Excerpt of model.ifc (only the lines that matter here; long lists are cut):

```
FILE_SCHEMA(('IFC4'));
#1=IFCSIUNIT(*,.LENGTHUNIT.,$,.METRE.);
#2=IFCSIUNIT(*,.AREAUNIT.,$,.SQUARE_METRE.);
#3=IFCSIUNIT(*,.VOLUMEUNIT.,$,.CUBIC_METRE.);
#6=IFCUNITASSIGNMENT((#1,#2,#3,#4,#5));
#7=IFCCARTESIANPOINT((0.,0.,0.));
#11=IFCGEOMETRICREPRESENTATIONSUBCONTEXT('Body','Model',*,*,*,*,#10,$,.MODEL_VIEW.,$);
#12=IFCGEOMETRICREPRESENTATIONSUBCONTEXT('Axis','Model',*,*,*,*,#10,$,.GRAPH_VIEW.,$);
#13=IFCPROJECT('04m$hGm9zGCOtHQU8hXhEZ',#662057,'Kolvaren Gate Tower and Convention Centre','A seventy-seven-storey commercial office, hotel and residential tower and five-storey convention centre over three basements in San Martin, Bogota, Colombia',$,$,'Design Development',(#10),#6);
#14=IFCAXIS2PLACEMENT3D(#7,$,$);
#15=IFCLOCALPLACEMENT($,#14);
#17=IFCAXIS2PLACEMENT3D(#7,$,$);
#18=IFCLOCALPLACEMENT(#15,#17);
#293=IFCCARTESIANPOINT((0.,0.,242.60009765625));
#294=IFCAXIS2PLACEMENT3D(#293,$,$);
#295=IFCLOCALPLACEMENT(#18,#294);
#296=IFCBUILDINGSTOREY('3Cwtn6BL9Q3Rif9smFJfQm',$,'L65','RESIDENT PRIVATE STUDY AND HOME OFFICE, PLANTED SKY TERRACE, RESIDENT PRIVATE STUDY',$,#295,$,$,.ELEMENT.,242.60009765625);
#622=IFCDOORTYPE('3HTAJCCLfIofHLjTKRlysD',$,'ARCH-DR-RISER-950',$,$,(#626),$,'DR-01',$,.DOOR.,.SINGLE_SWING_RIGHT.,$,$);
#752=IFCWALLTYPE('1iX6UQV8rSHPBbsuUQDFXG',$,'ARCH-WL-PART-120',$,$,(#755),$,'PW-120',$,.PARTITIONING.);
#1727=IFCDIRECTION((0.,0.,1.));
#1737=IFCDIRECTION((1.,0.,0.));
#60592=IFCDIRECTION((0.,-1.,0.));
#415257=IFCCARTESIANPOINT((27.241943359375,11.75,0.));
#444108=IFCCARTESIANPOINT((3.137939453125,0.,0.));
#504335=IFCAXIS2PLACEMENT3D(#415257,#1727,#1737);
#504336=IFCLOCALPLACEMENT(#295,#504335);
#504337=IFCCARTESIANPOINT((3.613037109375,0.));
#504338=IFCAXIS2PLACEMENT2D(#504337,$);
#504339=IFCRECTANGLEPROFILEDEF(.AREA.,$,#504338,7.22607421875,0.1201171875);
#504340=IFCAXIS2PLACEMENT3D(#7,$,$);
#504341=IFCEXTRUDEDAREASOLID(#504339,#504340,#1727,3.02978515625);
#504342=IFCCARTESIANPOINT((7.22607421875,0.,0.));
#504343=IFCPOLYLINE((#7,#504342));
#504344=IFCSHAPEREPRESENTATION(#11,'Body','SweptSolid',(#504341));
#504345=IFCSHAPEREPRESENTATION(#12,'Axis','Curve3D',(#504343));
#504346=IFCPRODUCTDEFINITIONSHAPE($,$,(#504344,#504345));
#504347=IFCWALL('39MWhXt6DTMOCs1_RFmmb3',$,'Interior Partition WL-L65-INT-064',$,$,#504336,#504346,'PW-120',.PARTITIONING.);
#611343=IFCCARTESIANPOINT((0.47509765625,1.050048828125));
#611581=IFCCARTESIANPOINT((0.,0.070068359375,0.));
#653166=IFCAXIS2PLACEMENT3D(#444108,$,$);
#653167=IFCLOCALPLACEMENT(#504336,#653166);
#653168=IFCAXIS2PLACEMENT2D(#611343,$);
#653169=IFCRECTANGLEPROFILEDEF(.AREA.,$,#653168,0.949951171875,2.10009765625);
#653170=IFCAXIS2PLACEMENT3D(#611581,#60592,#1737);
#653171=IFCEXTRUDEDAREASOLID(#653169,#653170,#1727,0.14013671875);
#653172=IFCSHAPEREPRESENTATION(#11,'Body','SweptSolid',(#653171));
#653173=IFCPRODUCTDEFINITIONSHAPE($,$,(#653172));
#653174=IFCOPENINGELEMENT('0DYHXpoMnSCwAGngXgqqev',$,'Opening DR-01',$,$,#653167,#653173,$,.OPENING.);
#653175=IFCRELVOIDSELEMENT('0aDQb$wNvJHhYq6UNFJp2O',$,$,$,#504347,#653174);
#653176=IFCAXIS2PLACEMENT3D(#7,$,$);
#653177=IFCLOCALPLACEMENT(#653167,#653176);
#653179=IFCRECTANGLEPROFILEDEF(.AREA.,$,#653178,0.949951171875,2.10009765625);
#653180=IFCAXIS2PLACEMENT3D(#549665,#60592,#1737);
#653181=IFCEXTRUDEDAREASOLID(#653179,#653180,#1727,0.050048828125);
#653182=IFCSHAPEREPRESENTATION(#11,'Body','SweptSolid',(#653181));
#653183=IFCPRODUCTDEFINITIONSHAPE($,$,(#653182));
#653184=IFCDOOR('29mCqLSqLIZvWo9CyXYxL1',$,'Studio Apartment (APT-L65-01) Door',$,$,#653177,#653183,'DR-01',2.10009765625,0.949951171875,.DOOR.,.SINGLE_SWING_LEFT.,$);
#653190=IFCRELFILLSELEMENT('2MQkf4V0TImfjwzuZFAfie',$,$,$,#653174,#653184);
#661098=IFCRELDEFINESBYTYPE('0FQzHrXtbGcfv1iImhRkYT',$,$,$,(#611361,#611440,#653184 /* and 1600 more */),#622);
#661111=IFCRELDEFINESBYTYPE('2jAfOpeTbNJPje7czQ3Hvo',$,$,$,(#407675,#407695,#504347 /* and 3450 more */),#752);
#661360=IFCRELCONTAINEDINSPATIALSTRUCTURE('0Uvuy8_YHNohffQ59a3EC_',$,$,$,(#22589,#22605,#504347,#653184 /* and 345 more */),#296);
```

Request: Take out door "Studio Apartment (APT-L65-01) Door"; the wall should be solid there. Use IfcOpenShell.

```python
import ifcopenshell
import ifcopenshell.api.feature
import ifcopenshell.api.root
import ifcopenshell.geom
import ifcopenshell.util.shape

model = ifcopenshell.open("model.ifc")
settings = ifcopenshell.geom.settings()


def volume(element):
    """Net volume in cubic metres, openings subtracted."""
    shape = ifcopenshell.geom.create_shape(settings, element)
    return ifcopenshell.util.shape.get_volume(shape.geometry)


door = model.by_guid("29mCqLSqLIZvWo9CyXYxL1")
opening = door.FillsVoids[0].RelatingOpeningElement
wall = opening.VoidsElements[0].RelatingBuildingElement
before = volume(wall)

ifcopenshell.api.root.remove_product(model, product=door)
ifcopenshell.api.feature.remove_feature(model, feature=opening)

after = volume(wall)

print(f"wall volume {before:.3f} -> {after:.3f} m3")

model.write("model_updated.ifc")
```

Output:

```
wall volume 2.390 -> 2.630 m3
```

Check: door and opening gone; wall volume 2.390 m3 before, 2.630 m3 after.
